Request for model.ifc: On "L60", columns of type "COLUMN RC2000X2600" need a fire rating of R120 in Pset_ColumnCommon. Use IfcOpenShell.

First a look at what the model holds.

```python
import ifcopenshell
import ifcopenshell.util.element

model = ifcopenshell.open("model.ifc")
print(model.schema)
storey = next(s for s in model.by_type("IfcBuildingStorey") if s.Name == "L60")
columns = [e for e in ifcopenshell.util.element.get_decomposition(storey) if e.is_a("IfcColumn")]
seen = {}
for e in columns:
    element_type = ifcopenshell.util.element.get_type(e)
    key = (element_type.Name if element_type != e and element_type else None, ifcopenshell.util.element.get_pset(e, "Pset_ColumnCommon", "FireRating"))
    seen[key] = seen.get(key, 0) + 1
for (name, value), count in sorted(seen.items(), key=str):
    print(count, "x", name, "|", value)
```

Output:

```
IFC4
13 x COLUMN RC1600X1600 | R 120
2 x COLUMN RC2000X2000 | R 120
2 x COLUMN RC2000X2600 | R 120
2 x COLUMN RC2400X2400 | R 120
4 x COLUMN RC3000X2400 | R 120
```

```python
import ifcopenshell
import ifcopenshell.api.pset
import ifcopenshell.util.element

model = ifcopenshell.open("model.ifc")

storey = next(s for s in model.by_type("IfcBuildingStorey") if s.Name == "L60")
columns = [e for e in ifcopenshell.util.element.get_decomposition(storey) if e.is_a("IfcColumn")]

count = 0
for e in columns:
    element_type = ifcopenshell.util.element.get_type(e)
    if element_type in (None, e) or element_type.Name != "COLUMN RC2000X2600":
        continue
    found = ifcopenshell.util.element.get_pset(e, "Pset_ColumnCommon", should_inherit=False)
    if found:
        pset = model.by_id(found["id"])
        if len(ifcopenshell.util.element.get_elements_by_pset(pset)) > 1:
            pset = ifcopenshell.api.pset.unshare_pset(model, products=[e], pset=pset)[0]
    else:
        pset = ifcopenshell.api.pset.add_pset(model, product=e, name="Pset_ColumnCommon")
    ifcopenshell.api.pset.edit_pset(model, pset=pset, properties={"FireRating": "R120"})
    count += 1

print(count, "columns updated")

model.write("model_v2.ifc")
```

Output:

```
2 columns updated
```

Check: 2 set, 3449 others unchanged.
